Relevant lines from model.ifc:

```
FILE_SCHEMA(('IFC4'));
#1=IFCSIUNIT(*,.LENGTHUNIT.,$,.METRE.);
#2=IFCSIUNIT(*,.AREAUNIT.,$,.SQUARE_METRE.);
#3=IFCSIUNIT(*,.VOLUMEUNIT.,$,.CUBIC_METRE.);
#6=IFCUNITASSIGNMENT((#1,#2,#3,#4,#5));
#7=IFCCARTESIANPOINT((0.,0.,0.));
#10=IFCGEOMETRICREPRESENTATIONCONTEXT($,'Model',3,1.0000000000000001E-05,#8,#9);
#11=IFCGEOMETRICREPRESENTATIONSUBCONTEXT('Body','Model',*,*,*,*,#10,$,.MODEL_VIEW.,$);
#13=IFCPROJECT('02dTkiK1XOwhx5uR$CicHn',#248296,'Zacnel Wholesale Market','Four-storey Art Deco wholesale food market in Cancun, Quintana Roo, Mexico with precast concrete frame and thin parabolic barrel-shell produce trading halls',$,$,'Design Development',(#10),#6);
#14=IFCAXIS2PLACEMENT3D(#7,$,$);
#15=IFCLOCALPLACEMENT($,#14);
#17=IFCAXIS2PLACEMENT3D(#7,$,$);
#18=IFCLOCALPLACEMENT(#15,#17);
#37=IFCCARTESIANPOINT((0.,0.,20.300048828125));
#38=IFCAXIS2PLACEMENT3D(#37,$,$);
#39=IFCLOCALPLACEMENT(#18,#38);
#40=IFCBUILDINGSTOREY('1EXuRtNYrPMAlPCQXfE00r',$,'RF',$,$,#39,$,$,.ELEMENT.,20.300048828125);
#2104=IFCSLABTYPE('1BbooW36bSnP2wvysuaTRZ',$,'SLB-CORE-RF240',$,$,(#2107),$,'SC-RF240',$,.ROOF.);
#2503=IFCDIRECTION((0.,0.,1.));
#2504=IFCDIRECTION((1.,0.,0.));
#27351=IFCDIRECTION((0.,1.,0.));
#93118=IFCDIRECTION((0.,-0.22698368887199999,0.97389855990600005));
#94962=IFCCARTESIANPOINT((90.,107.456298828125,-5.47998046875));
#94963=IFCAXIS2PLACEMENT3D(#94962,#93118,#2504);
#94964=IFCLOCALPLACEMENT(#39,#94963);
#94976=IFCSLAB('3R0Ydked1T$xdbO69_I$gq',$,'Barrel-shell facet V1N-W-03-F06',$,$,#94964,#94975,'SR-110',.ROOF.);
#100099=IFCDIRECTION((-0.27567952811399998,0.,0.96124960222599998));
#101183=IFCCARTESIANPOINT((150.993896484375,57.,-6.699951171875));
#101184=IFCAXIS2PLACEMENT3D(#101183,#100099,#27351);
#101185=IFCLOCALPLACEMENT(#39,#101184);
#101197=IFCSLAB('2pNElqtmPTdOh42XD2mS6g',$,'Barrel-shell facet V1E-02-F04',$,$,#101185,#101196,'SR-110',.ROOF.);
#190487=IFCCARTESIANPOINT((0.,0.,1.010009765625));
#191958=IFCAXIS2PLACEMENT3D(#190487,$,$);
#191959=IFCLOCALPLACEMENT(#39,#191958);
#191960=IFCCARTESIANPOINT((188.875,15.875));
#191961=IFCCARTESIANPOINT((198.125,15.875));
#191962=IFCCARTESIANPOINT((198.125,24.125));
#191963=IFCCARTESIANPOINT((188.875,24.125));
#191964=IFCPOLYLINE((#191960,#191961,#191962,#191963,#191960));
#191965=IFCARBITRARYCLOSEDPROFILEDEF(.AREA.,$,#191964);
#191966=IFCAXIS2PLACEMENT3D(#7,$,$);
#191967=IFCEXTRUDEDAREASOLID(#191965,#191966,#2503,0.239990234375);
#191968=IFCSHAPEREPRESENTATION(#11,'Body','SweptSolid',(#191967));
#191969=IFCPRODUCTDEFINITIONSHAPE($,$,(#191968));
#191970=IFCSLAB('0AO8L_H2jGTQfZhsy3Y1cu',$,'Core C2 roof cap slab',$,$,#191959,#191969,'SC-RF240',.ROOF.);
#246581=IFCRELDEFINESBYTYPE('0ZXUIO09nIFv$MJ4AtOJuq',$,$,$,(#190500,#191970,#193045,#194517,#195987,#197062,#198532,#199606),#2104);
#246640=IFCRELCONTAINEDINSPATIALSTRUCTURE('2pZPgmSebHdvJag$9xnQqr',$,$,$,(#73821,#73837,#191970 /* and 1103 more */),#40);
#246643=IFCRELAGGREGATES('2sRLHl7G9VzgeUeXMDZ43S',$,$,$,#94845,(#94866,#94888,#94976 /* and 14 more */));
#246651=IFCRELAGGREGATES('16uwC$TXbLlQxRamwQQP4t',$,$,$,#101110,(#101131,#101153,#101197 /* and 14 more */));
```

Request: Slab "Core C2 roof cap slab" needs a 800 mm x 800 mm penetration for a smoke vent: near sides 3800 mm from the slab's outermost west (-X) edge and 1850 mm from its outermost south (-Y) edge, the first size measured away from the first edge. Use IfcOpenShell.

```python
import numpy as np
import ifcopenshell
import ifcopenshell.api.feature
import ifcopenshell.api.geometry
import ifcopenshell.api.root
import ifcopenshell.geom
import ifcopenshell.util.placement
import ifcopenshell.util.representation
import ifcopenshell.util.shape
import ifcopenshell.util.unit

model = ifcopenshell.open("model.ifc")
unit_scale = ifcopenshell.util.unit.calculate_unit_scale(model)
settings = ifcopenshell.geom.settings()


def volume(element):
    """Net volume in cubic metres, openings subtracted."""
    shape = ifcopenshell.geom.create_shape(settings, element)
    return ifcopenshell.util.shape.get_volume(shape.geometry)


slab = model.by_guid("0AO8L_H2jGTQfZhsy3Y1cu")
before = volume(slab)

# Extent in the slab's own axes, in metres. The edges named are its -X and -Y sides.
slab_shape = ifcopenshell.geom.create_shape(settings, slab)
vertices = ifcopenshell.util.shape.get_vertices(slab_shape.geometry)
x_min, y_min, bottom = vertices.min(axis=0)
top = vertices[:, 2].max()

opening = ifcopenshell.api.root.create_entity(model, ifc_class="IfcOpeningElement", name="Smoke vent opening", predefined_type="OPENING")
context = ifcopenshell.util.representation.get_context(model, "Model", "Body", "MODEL_VIEW")
width, depth = 0.8, 0.8
outline = [(0.0, 0.0), (width, 0.0), (width, depth), (0.0, depth), (0.0, 0.0)]
# Overshoot both faces by 50 mm so the cut is clean.
shape = ifcopenshell.api.geometry.add_slab_representation(
    model, context=context, depth=top - bottom + 0.1, polyline=outline
)
ifcopenshell.api.geometry.assign_representation(model, product=opening, representation=shape)

matrix = ifcopenshell.util.placement.get_local_placement(slab.ObjectPlacement)
matrix[:, 3] = matrix @ np.append(np.array([x_min + 3.8, y_min + 1.85, bottom - 0.05]) / unit_scale, 1.0)
ifcopenshell.api.geometry.edit_object_placement(model, product=opening, matrix=matrix, is_si=False)
ifcopenshell.api.feature.add_feature(model, feature=opening, element=slab)

after = volume(slab)

print(f"slab volume {before:.3f} -> {after:.3f} m3")

model.write("model_updated.ifc")
```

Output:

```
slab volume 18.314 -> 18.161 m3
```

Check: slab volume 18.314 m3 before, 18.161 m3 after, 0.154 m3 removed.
